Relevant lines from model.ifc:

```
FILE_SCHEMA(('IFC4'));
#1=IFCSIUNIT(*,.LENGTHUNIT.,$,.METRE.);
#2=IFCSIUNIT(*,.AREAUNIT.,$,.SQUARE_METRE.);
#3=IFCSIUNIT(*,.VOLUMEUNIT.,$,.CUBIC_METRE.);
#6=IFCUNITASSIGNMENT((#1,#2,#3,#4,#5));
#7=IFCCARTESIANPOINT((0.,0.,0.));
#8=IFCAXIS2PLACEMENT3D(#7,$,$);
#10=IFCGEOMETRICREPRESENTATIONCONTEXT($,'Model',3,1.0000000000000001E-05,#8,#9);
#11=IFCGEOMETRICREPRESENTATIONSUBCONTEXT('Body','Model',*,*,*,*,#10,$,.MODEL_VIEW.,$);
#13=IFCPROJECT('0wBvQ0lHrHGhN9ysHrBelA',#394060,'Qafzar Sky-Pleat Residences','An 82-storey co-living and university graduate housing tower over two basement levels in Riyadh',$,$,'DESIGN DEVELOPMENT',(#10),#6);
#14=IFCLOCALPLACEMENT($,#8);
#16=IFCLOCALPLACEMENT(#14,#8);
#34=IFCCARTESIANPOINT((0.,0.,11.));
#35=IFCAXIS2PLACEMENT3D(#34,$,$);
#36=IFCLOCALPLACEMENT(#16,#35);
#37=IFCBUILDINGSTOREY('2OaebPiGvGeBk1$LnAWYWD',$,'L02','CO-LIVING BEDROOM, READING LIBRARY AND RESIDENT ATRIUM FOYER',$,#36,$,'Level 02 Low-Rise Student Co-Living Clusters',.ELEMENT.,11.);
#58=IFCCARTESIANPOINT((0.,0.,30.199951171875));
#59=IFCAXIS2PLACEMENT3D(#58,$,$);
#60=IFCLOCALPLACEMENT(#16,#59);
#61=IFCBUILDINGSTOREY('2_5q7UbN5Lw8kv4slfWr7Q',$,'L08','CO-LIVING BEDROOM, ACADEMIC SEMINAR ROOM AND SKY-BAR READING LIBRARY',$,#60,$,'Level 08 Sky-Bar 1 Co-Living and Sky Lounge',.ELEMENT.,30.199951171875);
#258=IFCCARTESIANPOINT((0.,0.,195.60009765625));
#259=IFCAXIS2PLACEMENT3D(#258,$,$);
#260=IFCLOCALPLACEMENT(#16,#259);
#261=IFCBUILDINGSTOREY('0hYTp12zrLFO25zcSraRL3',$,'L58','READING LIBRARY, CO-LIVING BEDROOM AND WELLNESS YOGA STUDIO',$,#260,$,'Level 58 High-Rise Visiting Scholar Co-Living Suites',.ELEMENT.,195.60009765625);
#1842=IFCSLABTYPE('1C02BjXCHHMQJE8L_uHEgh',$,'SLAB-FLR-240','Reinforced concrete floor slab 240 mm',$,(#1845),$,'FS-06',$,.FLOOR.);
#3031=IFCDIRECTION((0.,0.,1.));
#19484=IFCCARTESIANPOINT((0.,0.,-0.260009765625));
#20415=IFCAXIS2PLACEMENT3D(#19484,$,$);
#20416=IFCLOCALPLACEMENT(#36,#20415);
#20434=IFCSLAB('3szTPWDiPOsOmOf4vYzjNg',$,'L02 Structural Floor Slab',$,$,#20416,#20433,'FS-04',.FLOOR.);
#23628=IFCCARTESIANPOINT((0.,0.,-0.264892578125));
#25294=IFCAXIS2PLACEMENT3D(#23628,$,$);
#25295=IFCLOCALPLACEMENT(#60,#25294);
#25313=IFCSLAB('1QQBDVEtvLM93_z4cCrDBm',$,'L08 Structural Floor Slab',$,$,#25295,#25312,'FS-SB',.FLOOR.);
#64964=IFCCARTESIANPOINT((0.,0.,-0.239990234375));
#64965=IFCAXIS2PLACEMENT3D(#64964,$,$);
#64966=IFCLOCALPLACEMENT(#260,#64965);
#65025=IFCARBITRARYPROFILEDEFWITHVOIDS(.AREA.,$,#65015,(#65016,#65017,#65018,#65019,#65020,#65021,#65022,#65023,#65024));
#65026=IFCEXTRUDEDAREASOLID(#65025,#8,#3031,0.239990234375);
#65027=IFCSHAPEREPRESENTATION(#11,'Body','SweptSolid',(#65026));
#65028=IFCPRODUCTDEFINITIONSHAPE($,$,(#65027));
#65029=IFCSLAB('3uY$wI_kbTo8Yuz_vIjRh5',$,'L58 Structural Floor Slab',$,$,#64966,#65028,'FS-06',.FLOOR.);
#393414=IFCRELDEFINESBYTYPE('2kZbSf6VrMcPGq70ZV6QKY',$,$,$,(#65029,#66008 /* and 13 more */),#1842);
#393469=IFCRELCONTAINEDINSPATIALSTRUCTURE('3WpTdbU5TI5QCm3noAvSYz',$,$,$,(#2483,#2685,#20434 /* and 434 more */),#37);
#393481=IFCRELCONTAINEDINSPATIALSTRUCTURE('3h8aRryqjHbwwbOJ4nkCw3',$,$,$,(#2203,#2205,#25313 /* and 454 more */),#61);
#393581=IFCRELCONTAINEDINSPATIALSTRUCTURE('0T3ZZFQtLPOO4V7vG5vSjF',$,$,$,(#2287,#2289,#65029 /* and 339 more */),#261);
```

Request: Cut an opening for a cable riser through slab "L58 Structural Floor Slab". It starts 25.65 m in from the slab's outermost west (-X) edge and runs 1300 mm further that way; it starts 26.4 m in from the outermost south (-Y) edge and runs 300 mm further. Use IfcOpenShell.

```python
import numpy as np
import ifcopenshell
import ifcopenshell.api.feature
import ifcopenshell.api.geometry
import ifcopenshell.api.root
import ifcopenshell.geom
import ifcopenshell.util.placement
import ifcopenshell.util.representation
import ifcopenshell.util.shape
import ifcopenshell.util.unit

model = ifcopenshell.open("model.ifc")
unit_scale = ifcopenshell.util.unit.calculate_unit_scale(model)
settings = ifcopenshell.geom.settings()


def volume(element):
    """Net volume in cubic metres, openings subtracted."""
    shape = ifcopenshell.geom.create_shape(settings, element)
    return ifcopenshell.util.shape.get_volume(shape.geometry)


slab = model.by_guid("3uY$wI_kbTo8Yuz_vIjRh5")
before = volume(slab)

# Extent in the slab's own axes, in metres. The edges named are its -X and -Y sides.
slab_shape = ifcopenshell.geom.create_shape(settings, slab)
vertices = ifcopenshell.util.shape.get_vertices(slab_shape.geometry)
x_min, y_min, bottom = vertices.min(axis=0)
top = vertices[:, 2].max()

opening = ifcopenshell.api.root.create_entity(model, ifc_class="IfcOpeningElement", name="Cable riser opening", predefined_type="OPENING")
context = ifcopenshell.util.representation.get_context(model, "Model", "Body", "MODEL_VIEW")
width, depth = 1.3, 0.3
outline = [(0.0, 0.0), (width, 0.0), (width, depth), (0.0, depth), (0.0, 0.0)]
# Overshoot both faces by 50 mm so the cut is clean.
shape = ifcopenshell.api.geometry.add_slab_representation(
    model, context=context, depth=top - bottom + 0.1, polyline=outline
)
ifcopenshell.api.geometry.assign_representation(model, product=opening, representation=shape)

matrix = ifcopenshell.util.placement.get_local_placement(slab.ObjectPlacement)
matrix[:, 3] = matrix @ np.append(np.array([x_min + 25.65, y_min + 26.4, bottom - 0.05]) / unit_scale, 1.0)
ifcopenshell.api.geometry.edit_object_placement(model, product=opening, matrix=matrix, is_si=False)
ifcopenshell.api.feature.add_feature(model, feature=opening, element=slab)

after = volume(slab)

print(f"slab volume {before:.3f} -> {after:.3f} m3")

model.write("model_v2.ifc")
```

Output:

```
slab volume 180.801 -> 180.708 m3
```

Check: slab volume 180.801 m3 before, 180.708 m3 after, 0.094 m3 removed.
